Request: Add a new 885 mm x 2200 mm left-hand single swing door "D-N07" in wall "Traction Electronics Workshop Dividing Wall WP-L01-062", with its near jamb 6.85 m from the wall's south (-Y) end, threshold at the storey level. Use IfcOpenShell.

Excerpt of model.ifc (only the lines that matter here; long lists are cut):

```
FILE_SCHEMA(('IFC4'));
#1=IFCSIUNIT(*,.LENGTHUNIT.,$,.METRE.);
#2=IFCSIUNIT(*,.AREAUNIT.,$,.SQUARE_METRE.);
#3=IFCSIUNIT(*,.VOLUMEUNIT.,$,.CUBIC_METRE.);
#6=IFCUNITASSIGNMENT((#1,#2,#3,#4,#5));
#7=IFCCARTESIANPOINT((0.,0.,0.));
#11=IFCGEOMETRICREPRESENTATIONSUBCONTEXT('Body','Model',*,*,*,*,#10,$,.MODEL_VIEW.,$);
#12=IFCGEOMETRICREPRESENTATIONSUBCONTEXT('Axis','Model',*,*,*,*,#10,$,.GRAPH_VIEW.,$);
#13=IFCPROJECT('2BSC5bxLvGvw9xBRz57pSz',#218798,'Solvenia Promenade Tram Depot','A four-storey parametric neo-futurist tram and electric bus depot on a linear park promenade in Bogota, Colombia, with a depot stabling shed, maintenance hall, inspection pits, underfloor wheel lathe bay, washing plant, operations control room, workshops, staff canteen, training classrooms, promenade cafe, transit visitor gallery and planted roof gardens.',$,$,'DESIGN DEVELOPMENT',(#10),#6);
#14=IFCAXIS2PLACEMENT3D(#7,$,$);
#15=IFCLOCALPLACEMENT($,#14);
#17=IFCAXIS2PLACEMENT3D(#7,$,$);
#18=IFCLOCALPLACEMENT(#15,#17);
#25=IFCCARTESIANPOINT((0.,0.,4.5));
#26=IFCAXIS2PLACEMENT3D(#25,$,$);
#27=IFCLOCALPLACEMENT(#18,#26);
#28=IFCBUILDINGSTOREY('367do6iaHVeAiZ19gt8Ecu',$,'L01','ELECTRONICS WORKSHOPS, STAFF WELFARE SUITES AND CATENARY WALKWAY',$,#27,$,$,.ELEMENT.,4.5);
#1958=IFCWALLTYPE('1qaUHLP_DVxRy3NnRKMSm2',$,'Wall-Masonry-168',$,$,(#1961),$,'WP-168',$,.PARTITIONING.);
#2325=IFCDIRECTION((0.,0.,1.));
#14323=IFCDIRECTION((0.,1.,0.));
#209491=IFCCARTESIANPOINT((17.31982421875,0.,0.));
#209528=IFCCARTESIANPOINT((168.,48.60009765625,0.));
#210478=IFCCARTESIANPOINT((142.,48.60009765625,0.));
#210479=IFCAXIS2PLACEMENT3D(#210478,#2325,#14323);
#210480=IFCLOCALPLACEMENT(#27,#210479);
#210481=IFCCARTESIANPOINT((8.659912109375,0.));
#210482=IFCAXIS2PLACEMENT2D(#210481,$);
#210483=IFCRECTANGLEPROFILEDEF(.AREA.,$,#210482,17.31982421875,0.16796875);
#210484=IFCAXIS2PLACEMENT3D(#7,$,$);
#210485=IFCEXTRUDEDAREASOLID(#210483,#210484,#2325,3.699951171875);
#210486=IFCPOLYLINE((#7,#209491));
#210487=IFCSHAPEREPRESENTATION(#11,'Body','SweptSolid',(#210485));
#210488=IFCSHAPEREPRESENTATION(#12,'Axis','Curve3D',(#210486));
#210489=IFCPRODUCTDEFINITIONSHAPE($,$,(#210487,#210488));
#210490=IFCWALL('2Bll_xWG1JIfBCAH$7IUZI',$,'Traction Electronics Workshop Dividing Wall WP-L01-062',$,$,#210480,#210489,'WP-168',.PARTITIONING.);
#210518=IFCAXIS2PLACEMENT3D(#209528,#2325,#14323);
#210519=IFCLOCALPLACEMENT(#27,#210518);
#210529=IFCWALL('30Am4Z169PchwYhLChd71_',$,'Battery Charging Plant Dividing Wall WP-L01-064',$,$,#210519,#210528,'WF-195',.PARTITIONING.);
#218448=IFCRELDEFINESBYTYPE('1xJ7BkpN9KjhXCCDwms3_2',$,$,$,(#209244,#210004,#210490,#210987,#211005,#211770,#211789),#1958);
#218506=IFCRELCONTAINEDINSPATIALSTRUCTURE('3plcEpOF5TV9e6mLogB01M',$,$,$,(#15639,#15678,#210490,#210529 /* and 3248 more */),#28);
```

```python
import numpy as np
import ifcopenshell
import ifcopenshell.api.feature
import ifcopenshell.api.geometry
import ifcopenshell.api.root
import ifcopenshell.api.spatial
import ifcopenshell.geom
import ifcopenshell.util.element
import ifcopenshell.util.placement
import ifcopenshell.util.representation
import ifcopenshell.util.shape
import ifcopenshell.util.unit

model = ifcopenshell.open("model.ifc")
unit_scale = ifcopenshell.util.unit.calculate_unit_scale(model)
settings = ifcopenshell.geom.settings()


def volume(element):
    """Net volume in cubic metres, openings subtracted."""
    shape = ifcopenshell.geom.create_shape(settings, element)
    return ifcopenshell.util.shape.get_volume(shape.geometry)


wall = model.by_guid("2Bll_xWG1JIfBCAH$7IUZI")
storey = ifcopenshell.util.element.get_container(wall, ifc_class="IfcBuildingStorey")
context = ifcopenshell.util.representation.get_context(model, "Model", "Body", "MODEL_VIEW")
before = volume(wall)

width, height, from_end, sill = 0.885, 2.2, 6.85, 0.0  # metres

# The wall runs along its own X axis, and the end named is its -X end.
wall_shape = ifcopenshell.geom.create_shape(settings, wall)
x, y, z = ifcopenshell.util.shape.get_vertices(wall_shape.geometry).T
start = x.min() + from_end
face, thickness = float(y.min()), float(y.max() - y.min())
wall_matrix = ifcopenshell.util.placement.get_local_placement(wall.ObjectPlacement)
level = ifcopenshell.util.placement.get_local_placement(storey.ObjectPlacement)[2, 3]


def in_wall(x, y):
    """Placement at x, y metres in the wall's axes, at sill height."""
    matrix = wall_matrix.copy()
    matrix[:, 3] = wall_matrix @ np.array([x / unit_scale, y / unit_scale, 0.0, 1.0])
    matrix[2, 3] = level + sill / unit_scale
    return matrix


# Opening: a box that overshoots both wall faces by 50 mm.
opening = ifcopenshell.api.root.create_entity(model, ifc_class="IfcOpeningElement", predefined_type="OPENING")
box = ifcopenshell.api.geometry.add_wall_representation(
    model, context=context, length=width, height=height, thickness=thickness + 0.1
)
ifcopenshell.api.geometry.assign_representation(model, product=opening, representation=box)
ifcopenshell.api.geometry.edit_object_placement(model, product=opening, matrix=in_wall(start, face - 0.05), is_si=False)
ifcopenshell.api.feature.add_feature(model, feature=opening, element=wall)

door = ifcopenshell.api.root.create_entity(model, ifc_class="IfcDoor", name="D-N07", predefined_type="DOOR")
door.OverallWidth, door.OverallHeight = width / unit_scale, height / unit_scale
door.OperationType = "SINGLE_SWING_LEFT"
body = ifcopenshell.api.geometry.add_door_representation(
    model,
    context=context,
    overall_width=door.OverallWidth,
    overall_height=door.OverallHeight,
    operation_type="SINGLE_SWING_LEFT",
    lining_properties={"LiningDepth": thickness / unit_scale, "ThresholdDepth": thickness / unit_scale},
)
ifcopenshell.api.geometry.assign_representation(model, product=door, representation=body)
ifcopenshell.api.spatial.assign_container(model, products=[door], relating_structure=storey)
ifcopenshell.api.feature.add_filling(model, opening=opening, element=door)

# The lining spans the wall, so the door starts at the wall face.
ifcopenshell.api.geometry.edit_object_placement(model, product=door, matrix=in_wall(start, face), is_si=False)

after = volume(wall)

print(f"wall volume {before:.3f} -> {after:.3f} m3")

model.write("model_rev.ifc")
```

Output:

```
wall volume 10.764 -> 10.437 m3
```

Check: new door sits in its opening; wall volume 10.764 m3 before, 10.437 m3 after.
